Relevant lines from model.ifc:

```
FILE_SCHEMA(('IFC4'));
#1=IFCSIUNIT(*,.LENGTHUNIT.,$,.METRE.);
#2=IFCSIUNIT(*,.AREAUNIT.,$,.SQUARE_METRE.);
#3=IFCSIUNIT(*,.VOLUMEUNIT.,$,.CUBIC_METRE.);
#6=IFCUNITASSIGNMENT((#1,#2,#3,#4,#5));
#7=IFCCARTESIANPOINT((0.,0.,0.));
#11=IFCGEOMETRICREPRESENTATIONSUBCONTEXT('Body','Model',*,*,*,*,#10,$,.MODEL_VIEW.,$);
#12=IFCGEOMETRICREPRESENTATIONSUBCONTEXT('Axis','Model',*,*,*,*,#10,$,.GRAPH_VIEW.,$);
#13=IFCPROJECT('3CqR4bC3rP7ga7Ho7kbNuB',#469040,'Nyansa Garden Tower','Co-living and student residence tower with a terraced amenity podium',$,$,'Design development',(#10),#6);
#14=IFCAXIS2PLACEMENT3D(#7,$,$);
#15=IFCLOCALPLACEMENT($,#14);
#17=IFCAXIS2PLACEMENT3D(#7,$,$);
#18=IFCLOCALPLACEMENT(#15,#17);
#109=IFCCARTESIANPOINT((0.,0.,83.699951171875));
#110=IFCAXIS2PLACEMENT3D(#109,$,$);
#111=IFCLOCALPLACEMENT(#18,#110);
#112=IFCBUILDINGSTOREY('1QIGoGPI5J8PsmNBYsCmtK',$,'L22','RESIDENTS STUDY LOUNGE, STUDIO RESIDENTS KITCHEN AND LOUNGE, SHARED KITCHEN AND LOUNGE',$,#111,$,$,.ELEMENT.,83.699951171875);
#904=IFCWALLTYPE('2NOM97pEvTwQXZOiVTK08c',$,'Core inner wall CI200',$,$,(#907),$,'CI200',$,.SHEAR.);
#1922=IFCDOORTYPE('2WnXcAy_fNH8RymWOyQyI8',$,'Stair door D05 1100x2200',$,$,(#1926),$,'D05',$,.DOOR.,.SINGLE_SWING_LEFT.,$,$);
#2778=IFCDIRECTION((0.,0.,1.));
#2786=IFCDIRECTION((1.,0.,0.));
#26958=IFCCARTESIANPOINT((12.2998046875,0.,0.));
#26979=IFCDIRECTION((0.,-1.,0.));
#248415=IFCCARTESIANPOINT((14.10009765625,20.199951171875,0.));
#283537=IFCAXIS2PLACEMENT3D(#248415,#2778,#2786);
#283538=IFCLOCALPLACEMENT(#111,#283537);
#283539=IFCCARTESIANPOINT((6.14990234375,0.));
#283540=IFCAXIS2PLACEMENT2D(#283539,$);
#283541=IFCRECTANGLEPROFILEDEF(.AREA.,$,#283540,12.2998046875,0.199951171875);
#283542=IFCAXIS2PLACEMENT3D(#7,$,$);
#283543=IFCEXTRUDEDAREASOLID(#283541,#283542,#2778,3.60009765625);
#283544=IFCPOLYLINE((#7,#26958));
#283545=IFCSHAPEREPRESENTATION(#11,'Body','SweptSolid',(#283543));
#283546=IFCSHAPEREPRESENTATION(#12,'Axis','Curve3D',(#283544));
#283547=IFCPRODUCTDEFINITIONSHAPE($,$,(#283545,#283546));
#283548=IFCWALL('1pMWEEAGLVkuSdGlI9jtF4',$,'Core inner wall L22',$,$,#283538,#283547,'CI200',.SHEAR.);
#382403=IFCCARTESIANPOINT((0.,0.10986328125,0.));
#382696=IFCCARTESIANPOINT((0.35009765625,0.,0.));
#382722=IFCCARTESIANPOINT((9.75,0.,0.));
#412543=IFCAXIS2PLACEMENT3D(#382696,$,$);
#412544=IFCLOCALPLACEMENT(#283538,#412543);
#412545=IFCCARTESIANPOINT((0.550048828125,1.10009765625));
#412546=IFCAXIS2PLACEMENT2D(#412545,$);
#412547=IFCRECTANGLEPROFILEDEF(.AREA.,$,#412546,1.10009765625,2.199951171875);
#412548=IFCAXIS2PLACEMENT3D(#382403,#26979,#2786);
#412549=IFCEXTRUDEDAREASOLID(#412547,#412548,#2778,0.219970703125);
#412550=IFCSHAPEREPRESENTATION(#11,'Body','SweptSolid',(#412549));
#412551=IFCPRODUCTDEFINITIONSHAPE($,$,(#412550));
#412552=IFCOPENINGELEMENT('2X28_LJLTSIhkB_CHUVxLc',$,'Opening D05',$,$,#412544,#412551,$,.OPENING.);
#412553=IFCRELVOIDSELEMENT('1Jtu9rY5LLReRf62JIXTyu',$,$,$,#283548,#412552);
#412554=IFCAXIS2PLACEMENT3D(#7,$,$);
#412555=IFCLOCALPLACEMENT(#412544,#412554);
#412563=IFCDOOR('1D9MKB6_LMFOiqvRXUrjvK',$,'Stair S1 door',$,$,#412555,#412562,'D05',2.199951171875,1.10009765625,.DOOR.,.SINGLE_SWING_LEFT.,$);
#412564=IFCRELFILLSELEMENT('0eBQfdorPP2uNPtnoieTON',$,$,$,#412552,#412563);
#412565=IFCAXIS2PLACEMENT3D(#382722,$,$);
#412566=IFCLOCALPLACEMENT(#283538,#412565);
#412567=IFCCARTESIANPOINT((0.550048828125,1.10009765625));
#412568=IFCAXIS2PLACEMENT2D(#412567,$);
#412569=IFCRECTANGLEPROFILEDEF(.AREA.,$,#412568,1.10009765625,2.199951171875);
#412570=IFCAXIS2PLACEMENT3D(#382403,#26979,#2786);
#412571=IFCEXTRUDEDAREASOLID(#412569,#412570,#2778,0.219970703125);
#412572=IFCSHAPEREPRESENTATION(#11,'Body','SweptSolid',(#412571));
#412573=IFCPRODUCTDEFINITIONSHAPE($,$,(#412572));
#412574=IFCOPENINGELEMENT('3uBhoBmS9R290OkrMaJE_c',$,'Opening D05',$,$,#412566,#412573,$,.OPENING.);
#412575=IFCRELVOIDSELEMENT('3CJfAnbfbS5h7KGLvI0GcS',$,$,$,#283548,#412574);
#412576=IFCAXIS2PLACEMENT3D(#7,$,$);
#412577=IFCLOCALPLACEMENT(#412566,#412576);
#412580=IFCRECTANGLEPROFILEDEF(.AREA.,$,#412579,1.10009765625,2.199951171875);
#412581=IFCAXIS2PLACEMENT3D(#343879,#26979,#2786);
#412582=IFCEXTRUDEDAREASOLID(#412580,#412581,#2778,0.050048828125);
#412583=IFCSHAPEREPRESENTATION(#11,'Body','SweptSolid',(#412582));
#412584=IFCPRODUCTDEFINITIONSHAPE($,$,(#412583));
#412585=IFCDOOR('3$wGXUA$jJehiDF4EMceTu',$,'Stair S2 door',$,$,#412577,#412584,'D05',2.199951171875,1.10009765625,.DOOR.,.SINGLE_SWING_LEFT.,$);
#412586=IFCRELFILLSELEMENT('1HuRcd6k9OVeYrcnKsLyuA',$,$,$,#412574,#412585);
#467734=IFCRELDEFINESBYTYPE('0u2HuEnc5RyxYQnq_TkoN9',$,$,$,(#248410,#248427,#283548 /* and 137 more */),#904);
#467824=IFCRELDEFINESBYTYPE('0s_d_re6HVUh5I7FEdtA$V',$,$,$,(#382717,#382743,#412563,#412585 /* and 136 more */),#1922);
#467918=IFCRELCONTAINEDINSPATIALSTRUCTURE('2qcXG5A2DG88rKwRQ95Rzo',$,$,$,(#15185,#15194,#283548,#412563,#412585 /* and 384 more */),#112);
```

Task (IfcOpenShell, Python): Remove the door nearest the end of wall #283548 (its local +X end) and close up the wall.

```python
import ifcopenshell
import ifcopenshell.api.feature
import ifcopenshell.api.root
import ifcopenshell.geom
import ifcopenshell.util.shape

model = ifcopenshell.open("model.ifc")
settings = ifcopenshell.geom.settings()


def volume(element):
    """Net volume in cubic metres, openings subtracted."""
    shape = ifcopenshell.geom.create_shape(settings, element)
    return ifcopenshell.util.shape.get_volume(shape.geometry)


door = model.by_guid("3$wGXUA$jJehiDF4EMceTu")
opening = door.FillsVoids[0].RelatingOpeningElement
wall = opening.VoidsElements[0].RelatingBuildingElement
before = volume(wall)

ifcopenshell.api.root.remove_product(model, product=door)
ifcopenshell.api.feature.remove_feature(model, feature=opening)

after = volume(wall)

print(f"wall volume {before:.3f} -> {after:.3f} m3")

model.write("model_edited.ifc")
```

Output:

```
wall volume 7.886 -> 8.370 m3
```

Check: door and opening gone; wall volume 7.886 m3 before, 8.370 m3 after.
